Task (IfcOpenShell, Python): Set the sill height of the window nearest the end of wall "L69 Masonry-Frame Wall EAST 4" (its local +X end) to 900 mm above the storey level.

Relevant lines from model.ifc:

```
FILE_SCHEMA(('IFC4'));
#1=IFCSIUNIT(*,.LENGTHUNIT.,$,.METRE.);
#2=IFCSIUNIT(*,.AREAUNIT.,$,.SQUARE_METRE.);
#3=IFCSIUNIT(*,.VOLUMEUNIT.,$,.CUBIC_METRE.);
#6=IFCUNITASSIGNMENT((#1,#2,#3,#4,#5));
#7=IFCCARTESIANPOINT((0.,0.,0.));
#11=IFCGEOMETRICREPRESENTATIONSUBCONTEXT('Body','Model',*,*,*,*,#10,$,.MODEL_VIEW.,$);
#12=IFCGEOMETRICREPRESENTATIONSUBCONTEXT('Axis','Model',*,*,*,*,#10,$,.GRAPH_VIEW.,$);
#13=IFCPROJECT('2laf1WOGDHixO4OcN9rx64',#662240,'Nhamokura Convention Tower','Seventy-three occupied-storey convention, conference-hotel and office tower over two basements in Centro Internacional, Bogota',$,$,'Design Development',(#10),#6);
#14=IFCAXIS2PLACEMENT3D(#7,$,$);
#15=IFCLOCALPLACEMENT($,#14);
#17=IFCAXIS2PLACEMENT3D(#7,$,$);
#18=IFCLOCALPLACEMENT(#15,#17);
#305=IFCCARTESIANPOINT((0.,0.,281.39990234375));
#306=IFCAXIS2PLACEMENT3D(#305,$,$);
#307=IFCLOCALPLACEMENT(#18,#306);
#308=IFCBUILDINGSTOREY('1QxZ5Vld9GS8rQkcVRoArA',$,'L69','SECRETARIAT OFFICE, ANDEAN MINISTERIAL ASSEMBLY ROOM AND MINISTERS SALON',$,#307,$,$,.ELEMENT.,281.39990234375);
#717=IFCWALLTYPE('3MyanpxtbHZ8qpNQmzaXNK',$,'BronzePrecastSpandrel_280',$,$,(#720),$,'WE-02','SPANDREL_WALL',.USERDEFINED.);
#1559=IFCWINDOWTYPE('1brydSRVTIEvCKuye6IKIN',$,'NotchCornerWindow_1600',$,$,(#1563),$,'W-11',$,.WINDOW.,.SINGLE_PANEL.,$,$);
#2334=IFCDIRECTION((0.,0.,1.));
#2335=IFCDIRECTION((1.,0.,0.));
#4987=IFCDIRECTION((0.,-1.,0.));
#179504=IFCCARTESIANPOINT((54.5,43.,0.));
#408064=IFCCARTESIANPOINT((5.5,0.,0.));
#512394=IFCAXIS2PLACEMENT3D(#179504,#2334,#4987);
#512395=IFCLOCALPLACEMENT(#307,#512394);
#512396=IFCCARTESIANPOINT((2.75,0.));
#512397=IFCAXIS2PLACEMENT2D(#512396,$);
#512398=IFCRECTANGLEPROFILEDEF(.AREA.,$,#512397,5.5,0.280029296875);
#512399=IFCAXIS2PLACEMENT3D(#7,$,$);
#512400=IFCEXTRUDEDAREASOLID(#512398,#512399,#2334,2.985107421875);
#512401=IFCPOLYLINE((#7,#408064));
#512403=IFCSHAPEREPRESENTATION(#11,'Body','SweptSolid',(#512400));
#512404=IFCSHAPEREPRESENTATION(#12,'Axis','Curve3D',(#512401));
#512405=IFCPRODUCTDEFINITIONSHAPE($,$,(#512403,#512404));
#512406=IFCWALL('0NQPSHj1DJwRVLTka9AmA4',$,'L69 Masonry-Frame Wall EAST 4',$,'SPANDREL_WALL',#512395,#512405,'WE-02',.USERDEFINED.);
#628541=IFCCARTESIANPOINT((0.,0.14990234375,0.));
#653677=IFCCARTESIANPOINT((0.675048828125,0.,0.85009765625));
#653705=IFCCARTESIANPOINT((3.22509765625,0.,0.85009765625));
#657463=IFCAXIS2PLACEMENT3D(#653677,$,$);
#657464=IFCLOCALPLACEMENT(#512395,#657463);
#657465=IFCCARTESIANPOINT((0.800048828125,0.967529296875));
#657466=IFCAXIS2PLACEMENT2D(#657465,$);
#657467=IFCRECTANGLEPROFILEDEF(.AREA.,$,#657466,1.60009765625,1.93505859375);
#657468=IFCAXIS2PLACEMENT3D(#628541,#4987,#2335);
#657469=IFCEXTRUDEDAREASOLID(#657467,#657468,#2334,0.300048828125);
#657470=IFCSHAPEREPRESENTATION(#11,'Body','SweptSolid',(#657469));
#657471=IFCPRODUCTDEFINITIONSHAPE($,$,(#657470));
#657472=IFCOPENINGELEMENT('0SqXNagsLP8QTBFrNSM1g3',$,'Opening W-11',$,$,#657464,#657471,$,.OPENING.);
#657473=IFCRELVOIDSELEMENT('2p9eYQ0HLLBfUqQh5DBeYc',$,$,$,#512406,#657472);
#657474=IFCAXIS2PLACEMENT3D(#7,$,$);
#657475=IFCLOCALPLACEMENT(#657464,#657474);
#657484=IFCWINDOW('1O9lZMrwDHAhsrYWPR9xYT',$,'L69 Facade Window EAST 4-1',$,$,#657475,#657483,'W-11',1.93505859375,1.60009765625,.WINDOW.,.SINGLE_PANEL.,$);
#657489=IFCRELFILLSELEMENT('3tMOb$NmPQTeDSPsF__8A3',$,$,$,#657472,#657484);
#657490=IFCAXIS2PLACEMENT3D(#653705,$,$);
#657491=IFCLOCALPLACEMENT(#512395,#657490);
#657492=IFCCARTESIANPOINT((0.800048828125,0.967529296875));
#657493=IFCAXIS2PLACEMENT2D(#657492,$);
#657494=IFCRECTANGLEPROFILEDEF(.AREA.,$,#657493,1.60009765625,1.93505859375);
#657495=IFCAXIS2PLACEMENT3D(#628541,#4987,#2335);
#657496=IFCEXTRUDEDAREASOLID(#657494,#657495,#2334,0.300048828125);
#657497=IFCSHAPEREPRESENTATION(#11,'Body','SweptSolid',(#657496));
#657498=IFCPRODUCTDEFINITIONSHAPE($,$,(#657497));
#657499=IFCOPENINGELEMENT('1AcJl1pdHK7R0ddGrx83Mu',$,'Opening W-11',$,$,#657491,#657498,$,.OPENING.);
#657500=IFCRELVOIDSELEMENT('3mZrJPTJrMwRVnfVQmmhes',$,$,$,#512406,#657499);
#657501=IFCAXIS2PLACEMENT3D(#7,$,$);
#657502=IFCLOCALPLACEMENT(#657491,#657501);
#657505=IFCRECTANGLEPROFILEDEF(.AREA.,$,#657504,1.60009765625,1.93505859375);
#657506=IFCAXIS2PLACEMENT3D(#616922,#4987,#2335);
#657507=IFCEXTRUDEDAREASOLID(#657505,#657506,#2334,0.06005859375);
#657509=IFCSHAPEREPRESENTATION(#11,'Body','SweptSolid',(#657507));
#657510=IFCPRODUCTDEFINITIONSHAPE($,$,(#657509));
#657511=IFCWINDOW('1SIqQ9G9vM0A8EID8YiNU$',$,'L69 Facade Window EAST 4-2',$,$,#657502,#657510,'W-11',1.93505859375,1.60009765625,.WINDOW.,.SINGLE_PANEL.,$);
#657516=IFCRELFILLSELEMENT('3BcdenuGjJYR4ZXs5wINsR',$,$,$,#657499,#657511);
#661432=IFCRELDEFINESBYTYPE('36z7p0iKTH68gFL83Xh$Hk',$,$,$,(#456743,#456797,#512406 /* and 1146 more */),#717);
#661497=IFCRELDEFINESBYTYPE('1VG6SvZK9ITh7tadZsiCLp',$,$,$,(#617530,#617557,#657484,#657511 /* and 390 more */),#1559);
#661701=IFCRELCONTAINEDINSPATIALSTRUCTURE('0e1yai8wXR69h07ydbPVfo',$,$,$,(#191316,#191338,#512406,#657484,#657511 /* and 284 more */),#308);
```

```python
import numpy as np
import ifcopenshell
import ifcopenshell.api.geometry
import ifcopenshell.geom
import ifcopenshell.util.element
import ifcopenshell.util.placement
import ifcopenshell.util.shape
import ifcopenshell.util.unit

model = ifcopenshell.open("model.ifc")
unit_scale = ifcopenshell.util.unit.calculate_unit_scale(model)

window = model.by_guid("1SIqQ9G9vM0A8EID8YiNU$")
opening = window.FillsVoids[0].RelatingOpeningElement
storey = ifcopenshell.util.element.get_container(window, ifc_class="IfcBuildingStorey")
level = ifcopenshell.util.placement.get_local_placement(storey.ObjectPlacement)[2, 3]

# The opening's origin need not be at the sill, so measure its lowest point.
shape = ifcopenshell.geom.create_shape(ifcopenshell.geom.settings(), opening)
bottom = ifcopenshell.util.shape.get_shape_bottom_elevation(shape, shape.geometry) / unit_scale
dz = level + 0.9 / unit_scale - bottom

shift = np.array([0.0, 0.0, dz])
# The window is placed relative to its opening, so it follows when the opening moves.
matrix = ifcopenshell.util.placement.get_local_placement(opening.ObjectPlacement)
matrix[:3, 3] += shift
ifcopenshell.api.geometry.edit_object_placement(
    model, product=opening, matrix=matrix, is_si=False, should_transform_children=True
)

print(f"moved by {dz * unit_scale:+.3f} m")

model.write("model_edited.ifc")
```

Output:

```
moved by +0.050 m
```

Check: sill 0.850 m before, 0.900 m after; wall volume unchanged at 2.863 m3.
